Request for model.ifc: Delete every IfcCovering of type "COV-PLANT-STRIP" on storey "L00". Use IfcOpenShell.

First a look at what the model holds.

```python
import ifcopenshell
import ifcopenshell.util.element

model = ifcopenshell.open("model.ifc")
print(model.schema)
storey = next(s for s in model.by_type("IfcBuildingStorey") if s.Name == "L00")
coverings = [e for e in ifcopenshell.util.element.get_decomposition(storey) if e.is_a("IfcCovering")]
seen = {}
for e in coverings:
    element_type = ifcopenshell.util.element.get_type(e)
    name = element_type.Name if element_type not in (None, e) else None
    seen[name] = seen.get(name, 0) + 1
for name, count in sorted(seen.items(), key=str):
    print(count, "x", name)
```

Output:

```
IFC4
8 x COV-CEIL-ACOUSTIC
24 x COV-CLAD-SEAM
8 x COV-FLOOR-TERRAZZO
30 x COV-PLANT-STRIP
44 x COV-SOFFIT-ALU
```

```python
import ifcopenshell
import ifcopenshell.api.root
import ifcopenshell.util.element

model = ifcopenshell.open("model.ifc")

storey = next(s for s in model.by_type("IfcBuildingStorey") if s.Name == "L00")
coverings = [e for e in ifcopenshell.util.element.get_decomposition(storey) if e.is_a("IfcCovering")]
targets = [e for e in coverings if (t := ifcopenshell.util.element.get_type(e)) not in (None, e) and t.Name == "COV-PLANT-STRIP"]

for e in targets:
    ifcopenshell.api.root.remove_product(model, product=e)
print(len(targets), "removed")

model.write("model_rev.ifc")
```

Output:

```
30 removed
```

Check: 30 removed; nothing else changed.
